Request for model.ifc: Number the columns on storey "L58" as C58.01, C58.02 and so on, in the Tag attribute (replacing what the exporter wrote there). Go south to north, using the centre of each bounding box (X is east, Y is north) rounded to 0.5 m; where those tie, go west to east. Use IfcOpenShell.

First a look at what the model holds.

```python
import ifcopenshell
import ifcopenshell.util.element
import ifcopenshell.util.placement

model = ifcopenshell.open("model.ifc")
print(model.schema)
storey = next(s for s in model.by_type("IfcBuildingStorey") if s.Name == "L58")
columns = [e for e in ifcopenshell.util.element.get_decomposition(storey) if e.is_a("IfcColumn")]
for e in sorted(columns, key=lambda e: e.id()):
    origin = ifcopenshell.util.placement.get_local_placement(e.ObjectPlacement)[:3, 3]
    print(e.id(), e.Tag, e.Name, origin.round(2) + 0.0, sep=" | ")
```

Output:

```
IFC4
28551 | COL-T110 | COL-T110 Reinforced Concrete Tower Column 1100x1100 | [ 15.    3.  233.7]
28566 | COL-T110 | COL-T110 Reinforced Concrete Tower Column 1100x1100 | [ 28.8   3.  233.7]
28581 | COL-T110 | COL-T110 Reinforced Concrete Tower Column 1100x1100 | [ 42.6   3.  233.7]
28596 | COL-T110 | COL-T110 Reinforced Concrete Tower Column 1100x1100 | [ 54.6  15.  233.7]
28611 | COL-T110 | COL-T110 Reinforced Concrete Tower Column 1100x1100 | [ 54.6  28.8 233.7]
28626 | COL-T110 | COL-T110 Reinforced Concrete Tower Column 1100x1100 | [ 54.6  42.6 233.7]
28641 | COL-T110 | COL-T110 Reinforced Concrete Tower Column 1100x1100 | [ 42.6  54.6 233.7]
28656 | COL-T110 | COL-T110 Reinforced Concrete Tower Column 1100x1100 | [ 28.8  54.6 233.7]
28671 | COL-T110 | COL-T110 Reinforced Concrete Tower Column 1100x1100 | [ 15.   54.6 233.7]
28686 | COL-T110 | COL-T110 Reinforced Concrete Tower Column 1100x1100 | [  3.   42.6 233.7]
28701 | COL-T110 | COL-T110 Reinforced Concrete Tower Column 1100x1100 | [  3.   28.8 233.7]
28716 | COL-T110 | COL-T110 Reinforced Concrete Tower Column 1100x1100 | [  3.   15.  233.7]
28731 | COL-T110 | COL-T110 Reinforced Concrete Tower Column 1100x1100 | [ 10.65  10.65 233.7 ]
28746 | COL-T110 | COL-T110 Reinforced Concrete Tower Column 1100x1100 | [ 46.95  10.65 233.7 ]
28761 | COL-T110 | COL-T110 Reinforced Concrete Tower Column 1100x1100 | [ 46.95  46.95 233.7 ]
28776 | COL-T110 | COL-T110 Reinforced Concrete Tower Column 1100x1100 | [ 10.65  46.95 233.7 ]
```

```python
import ifcopenshell
import ifcopenshell.geom
import ifcopenshell.util.element
import ifcopenshell.util.shape

model = ifcopenshell.open("model.ifc")
settings = ifcopenshell.geom.settings()
settings.set("use-world-coords", True)


def centre(element):
    shape = ifcopenshell.geom.create_shape(settings, element)
    return ifcopenshell.util.shape.get_bbox_centroid(shape.geometry)


storey = next(s for s in model.by_type("IfcBuildingStorey") if s.Name == "L58")
columns = [e for e in ifcopenshell.util.element.get_decomposition(storey) if e.is_a("IfcColumn")]

# Insertion points can sit at a corner or the storey origin, so sort by the geometry (in metres).
centres = {e: centre(e) for e in columns}
columns.sort(key=lambda e: (round(centres[e][1] / 0.5), centres[e][0]))

for i, e in enumerate(columns, start=1):
    number = f"C58.{i:02d}"
    e.Tag = number
    print(e.id(), number)

model.write("model_rev.ifc")
```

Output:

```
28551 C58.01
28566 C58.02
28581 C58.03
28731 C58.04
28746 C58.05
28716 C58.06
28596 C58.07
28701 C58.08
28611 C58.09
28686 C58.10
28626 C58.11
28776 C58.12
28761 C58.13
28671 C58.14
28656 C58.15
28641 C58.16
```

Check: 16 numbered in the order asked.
